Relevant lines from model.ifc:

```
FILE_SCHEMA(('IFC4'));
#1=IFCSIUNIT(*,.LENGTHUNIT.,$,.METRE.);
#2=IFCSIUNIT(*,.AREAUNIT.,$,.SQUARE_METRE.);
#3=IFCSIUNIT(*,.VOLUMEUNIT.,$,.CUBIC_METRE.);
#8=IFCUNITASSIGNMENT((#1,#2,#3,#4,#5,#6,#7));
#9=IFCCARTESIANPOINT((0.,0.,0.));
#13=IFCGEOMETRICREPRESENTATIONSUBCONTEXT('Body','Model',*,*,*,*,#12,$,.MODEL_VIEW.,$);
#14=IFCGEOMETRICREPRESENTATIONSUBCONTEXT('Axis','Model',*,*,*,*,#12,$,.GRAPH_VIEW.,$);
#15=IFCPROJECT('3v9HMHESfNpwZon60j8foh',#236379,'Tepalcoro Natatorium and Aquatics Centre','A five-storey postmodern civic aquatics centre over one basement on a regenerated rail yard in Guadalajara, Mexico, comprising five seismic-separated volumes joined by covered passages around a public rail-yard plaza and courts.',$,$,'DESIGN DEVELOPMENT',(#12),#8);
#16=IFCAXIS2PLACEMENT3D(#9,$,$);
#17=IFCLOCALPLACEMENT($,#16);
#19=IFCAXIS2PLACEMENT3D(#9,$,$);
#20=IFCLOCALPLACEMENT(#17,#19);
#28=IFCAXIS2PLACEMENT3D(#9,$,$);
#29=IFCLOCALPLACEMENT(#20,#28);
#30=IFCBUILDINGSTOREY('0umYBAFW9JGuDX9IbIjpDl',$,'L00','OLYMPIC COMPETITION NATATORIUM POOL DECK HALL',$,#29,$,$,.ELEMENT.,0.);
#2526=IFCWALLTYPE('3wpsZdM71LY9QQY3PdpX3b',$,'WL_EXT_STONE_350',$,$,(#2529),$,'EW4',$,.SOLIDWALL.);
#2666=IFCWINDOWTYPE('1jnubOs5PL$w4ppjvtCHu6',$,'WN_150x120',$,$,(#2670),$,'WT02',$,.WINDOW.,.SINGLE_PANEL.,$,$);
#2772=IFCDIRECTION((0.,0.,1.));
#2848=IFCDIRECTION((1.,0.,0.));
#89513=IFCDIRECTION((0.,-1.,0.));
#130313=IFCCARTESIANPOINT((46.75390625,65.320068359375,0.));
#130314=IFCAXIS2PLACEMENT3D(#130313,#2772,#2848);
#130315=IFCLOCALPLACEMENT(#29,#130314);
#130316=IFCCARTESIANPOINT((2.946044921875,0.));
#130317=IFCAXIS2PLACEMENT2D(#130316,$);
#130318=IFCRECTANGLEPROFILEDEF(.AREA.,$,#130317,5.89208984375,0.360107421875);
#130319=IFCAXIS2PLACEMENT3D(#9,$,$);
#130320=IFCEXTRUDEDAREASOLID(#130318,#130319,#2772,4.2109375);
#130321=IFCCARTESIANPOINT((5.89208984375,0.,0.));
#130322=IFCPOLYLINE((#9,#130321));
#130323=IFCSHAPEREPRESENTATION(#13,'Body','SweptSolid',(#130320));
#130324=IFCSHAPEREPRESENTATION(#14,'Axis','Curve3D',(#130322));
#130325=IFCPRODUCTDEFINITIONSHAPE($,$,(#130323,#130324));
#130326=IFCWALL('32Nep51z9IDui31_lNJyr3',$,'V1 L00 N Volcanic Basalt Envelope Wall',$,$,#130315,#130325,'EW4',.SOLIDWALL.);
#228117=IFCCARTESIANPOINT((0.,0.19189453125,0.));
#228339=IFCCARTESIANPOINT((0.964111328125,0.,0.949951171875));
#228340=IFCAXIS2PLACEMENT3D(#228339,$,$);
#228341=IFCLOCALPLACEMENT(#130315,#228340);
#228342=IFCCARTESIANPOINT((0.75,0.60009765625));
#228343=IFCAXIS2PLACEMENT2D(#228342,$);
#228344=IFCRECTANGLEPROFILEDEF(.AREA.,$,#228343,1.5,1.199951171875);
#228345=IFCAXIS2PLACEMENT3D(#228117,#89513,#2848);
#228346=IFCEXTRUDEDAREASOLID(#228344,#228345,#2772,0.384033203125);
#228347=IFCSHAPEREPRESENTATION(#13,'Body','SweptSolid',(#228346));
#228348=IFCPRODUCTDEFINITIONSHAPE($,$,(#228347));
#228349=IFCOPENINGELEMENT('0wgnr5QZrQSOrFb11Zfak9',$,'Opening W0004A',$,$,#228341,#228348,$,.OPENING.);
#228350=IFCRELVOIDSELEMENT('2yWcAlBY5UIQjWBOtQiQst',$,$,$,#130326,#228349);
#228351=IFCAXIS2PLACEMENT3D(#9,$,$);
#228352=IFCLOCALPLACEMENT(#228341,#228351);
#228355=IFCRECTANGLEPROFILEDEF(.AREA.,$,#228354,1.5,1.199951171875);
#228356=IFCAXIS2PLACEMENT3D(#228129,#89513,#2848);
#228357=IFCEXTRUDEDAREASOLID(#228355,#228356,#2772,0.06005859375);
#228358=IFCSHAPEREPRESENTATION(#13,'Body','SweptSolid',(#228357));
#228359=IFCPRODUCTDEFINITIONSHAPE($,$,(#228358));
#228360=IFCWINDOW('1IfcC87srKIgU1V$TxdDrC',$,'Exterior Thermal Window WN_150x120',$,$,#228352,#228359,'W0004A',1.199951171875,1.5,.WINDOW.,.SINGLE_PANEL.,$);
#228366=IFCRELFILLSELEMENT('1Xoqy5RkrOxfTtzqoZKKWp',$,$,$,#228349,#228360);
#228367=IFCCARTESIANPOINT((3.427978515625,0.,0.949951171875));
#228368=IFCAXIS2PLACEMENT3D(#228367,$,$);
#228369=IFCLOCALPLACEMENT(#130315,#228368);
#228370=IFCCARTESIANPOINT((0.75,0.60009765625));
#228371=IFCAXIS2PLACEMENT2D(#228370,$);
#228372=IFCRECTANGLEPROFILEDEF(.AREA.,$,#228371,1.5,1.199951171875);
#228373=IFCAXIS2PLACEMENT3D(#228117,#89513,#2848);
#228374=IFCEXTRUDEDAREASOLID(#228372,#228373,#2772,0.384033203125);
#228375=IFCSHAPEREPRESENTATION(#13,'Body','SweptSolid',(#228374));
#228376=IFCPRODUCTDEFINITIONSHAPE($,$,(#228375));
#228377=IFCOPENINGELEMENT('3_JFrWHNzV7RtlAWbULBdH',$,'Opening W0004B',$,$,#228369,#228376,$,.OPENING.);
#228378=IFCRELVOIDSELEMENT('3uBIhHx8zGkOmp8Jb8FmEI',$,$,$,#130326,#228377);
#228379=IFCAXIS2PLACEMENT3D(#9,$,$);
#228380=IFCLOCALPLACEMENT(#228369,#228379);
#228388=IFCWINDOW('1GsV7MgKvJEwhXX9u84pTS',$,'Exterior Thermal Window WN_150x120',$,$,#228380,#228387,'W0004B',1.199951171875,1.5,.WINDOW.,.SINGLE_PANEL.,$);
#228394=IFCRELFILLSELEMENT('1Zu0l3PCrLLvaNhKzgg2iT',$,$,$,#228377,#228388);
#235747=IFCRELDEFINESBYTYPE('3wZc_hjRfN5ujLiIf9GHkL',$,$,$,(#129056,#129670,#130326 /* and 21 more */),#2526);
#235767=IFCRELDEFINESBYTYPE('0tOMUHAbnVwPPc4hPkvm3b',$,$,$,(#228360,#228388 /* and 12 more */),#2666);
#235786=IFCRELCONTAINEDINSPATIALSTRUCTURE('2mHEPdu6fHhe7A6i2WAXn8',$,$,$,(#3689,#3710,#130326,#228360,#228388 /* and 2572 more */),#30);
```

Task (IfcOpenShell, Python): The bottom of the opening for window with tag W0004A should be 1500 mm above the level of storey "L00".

```python
import numpy as np
import ifcopenshell
import ifcopenshell.api.geometry
import ifcopenshell.geom
import ifcopenshell.util.element
import ifcopenshell.util.placement
import ifcopenshell.util.shape
import ifcopenshell.util.unit

model = ifcopenshell.open("model.ifc")
unit_scale = ifcopenshell.util.unit.calculate_unit_scale(model)

window = model.by_guid("1IfcC87srKIgU1V$TxdDrC")
opening = window.FillsVoids[0].RelatingOpeningElement
storey = ifcopenshell.util.element.get_container(window, ifc_class="IfcBuildingStorey")
level = ifcopenshell.util.placement.get_local_placement(storey.ObjectPlacement)[2, 3]

# The opening's origin need not be at the sill, so measure its lowest point.
shape = ifcopenshell.geom.create_shape(ifcopenshell.geom.settings(), opening)
bottom = ifcopenshell.util.shape.get_shape_bottom_elevation(shape, shape.geometry) / unit_scale
dz = level + 1.5 / unit_scale - bottom

shift = np.array([0.0, 0.0, dz])
# The window is placed relative to its opening, so it follows when the opening moves.
matrix = ifcopenshell.util.placement.get_local_placement(opening.ObjectPlacement)
matrix[:3, 3] += shift
ifcopenshell.api.geometry.edit_object_placement(
    model, product=opening, matrix=matrix, is_si=False, should_transform_children=True
)

print(f"moved by {dz * unit_scale:+.3f} m")

model.write("model_rev.ifc")
```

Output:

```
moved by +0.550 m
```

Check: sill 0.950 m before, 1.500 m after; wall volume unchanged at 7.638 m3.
